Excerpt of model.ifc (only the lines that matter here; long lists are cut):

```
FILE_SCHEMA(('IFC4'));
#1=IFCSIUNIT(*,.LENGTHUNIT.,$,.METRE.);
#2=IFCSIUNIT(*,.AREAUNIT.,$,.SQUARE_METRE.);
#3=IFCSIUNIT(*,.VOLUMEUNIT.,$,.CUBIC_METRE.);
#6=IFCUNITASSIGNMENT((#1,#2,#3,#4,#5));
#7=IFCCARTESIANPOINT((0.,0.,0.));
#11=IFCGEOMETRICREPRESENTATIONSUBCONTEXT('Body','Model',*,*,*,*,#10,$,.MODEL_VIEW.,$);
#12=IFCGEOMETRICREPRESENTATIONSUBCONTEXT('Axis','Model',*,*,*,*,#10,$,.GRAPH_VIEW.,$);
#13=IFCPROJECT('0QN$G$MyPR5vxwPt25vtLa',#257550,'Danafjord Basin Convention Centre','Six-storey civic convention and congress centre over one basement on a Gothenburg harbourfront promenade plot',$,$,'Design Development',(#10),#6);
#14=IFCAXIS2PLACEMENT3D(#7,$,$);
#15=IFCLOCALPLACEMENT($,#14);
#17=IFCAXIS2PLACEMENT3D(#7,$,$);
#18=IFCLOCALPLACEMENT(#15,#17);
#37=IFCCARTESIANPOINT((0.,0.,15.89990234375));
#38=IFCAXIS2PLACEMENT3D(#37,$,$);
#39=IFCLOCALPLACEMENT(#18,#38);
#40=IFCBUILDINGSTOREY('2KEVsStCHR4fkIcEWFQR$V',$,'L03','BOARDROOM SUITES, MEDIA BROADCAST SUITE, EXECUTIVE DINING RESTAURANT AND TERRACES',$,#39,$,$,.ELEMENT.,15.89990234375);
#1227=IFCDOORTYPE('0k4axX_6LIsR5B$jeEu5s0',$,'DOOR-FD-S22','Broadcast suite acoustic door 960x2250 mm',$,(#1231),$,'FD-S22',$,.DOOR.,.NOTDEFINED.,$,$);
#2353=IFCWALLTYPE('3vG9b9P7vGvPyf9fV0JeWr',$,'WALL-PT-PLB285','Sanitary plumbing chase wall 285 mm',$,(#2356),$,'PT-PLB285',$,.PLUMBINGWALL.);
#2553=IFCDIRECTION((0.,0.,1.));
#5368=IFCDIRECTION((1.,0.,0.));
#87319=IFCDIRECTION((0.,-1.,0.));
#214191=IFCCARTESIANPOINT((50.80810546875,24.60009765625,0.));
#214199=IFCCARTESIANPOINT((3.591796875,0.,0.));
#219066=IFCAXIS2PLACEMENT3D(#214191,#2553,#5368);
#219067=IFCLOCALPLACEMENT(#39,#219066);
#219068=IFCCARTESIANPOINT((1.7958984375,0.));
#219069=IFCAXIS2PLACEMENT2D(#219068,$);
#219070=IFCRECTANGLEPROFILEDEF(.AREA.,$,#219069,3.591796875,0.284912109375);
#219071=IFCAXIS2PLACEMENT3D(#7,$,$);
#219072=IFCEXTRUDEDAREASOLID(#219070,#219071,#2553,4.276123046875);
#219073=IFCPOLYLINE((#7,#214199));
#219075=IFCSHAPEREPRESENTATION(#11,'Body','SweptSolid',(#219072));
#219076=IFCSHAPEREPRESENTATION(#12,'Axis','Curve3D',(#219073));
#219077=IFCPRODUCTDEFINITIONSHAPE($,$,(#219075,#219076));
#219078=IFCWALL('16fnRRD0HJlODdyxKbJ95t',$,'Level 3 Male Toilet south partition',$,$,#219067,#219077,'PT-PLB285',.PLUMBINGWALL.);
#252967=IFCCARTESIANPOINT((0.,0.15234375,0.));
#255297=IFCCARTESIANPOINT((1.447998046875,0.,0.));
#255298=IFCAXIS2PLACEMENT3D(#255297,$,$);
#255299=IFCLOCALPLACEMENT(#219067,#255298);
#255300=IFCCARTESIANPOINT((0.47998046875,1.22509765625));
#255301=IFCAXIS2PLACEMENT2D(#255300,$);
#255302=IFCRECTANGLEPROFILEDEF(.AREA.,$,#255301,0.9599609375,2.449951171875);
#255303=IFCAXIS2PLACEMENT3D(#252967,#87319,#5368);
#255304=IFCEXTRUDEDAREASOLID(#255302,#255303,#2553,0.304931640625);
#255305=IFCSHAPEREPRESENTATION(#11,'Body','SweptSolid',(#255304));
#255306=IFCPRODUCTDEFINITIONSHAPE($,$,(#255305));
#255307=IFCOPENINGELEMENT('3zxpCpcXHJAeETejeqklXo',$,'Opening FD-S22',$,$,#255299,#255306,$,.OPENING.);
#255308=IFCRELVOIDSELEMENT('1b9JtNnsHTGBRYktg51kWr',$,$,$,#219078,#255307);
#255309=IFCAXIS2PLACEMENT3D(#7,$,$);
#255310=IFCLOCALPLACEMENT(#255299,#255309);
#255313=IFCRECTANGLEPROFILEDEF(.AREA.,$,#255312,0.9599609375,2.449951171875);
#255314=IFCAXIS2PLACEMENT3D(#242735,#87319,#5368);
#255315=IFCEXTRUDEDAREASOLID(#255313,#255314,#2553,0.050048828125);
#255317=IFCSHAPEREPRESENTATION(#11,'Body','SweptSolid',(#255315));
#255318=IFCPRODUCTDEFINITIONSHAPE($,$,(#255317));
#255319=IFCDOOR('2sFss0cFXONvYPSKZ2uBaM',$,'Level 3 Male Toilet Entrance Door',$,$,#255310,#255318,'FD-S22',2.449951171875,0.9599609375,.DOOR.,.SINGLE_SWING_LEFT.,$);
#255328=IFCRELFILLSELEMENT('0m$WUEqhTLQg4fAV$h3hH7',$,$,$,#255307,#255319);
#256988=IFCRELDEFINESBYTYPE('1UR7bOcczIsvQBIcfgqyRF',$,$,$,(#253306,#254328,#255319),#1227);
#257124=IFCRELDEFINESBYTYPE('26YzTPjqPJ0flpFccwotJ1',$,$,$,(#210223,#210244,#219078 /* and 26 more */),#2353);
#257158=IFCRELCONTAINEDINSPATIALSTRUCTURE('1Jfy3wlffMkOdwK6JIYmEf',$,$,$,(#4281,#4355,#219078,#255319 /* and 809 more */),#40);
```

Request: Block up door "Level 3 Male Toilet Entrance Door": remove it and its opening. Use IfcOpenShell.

```python
import ifcopenshell
import ifcopenshell.api.feature
import ifcopenshell.api.root
import ifcopenshell.geom
import ifcopenshell.util.shape

model = ifcopenshell.open("model.ifc")
settings = ifcopenshell.geom.settings()


def volume(element):
    """Net volume in cubic metres, openings subtracted."""
    shape = ifcopenshell.geom.create_shape(settings, element)
    return ifcopenshell.util.shape.get_volume(shape.geometry)


door = model.by_guid("2sFss0cFXONvYPSKZ2uBaM")
opening = door.FillsVoids[0].RelatingOpeningElement
wall = opening.VoidsElements[0].RelatingBuildingElement
before = volume(wall)

ifcopenshell.api.root.remove_product(model, product=door)
ifcopenshell.api.feature.remove_feature(model, feature=opening)

after = volume(wall)

print(f"wall volume {before:.3f} -> {after:.3f} m3")

model.write("model_rev.ifc")
```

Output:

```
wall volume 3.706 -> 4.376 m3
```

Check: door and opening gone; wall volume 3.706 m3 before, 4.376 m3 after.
